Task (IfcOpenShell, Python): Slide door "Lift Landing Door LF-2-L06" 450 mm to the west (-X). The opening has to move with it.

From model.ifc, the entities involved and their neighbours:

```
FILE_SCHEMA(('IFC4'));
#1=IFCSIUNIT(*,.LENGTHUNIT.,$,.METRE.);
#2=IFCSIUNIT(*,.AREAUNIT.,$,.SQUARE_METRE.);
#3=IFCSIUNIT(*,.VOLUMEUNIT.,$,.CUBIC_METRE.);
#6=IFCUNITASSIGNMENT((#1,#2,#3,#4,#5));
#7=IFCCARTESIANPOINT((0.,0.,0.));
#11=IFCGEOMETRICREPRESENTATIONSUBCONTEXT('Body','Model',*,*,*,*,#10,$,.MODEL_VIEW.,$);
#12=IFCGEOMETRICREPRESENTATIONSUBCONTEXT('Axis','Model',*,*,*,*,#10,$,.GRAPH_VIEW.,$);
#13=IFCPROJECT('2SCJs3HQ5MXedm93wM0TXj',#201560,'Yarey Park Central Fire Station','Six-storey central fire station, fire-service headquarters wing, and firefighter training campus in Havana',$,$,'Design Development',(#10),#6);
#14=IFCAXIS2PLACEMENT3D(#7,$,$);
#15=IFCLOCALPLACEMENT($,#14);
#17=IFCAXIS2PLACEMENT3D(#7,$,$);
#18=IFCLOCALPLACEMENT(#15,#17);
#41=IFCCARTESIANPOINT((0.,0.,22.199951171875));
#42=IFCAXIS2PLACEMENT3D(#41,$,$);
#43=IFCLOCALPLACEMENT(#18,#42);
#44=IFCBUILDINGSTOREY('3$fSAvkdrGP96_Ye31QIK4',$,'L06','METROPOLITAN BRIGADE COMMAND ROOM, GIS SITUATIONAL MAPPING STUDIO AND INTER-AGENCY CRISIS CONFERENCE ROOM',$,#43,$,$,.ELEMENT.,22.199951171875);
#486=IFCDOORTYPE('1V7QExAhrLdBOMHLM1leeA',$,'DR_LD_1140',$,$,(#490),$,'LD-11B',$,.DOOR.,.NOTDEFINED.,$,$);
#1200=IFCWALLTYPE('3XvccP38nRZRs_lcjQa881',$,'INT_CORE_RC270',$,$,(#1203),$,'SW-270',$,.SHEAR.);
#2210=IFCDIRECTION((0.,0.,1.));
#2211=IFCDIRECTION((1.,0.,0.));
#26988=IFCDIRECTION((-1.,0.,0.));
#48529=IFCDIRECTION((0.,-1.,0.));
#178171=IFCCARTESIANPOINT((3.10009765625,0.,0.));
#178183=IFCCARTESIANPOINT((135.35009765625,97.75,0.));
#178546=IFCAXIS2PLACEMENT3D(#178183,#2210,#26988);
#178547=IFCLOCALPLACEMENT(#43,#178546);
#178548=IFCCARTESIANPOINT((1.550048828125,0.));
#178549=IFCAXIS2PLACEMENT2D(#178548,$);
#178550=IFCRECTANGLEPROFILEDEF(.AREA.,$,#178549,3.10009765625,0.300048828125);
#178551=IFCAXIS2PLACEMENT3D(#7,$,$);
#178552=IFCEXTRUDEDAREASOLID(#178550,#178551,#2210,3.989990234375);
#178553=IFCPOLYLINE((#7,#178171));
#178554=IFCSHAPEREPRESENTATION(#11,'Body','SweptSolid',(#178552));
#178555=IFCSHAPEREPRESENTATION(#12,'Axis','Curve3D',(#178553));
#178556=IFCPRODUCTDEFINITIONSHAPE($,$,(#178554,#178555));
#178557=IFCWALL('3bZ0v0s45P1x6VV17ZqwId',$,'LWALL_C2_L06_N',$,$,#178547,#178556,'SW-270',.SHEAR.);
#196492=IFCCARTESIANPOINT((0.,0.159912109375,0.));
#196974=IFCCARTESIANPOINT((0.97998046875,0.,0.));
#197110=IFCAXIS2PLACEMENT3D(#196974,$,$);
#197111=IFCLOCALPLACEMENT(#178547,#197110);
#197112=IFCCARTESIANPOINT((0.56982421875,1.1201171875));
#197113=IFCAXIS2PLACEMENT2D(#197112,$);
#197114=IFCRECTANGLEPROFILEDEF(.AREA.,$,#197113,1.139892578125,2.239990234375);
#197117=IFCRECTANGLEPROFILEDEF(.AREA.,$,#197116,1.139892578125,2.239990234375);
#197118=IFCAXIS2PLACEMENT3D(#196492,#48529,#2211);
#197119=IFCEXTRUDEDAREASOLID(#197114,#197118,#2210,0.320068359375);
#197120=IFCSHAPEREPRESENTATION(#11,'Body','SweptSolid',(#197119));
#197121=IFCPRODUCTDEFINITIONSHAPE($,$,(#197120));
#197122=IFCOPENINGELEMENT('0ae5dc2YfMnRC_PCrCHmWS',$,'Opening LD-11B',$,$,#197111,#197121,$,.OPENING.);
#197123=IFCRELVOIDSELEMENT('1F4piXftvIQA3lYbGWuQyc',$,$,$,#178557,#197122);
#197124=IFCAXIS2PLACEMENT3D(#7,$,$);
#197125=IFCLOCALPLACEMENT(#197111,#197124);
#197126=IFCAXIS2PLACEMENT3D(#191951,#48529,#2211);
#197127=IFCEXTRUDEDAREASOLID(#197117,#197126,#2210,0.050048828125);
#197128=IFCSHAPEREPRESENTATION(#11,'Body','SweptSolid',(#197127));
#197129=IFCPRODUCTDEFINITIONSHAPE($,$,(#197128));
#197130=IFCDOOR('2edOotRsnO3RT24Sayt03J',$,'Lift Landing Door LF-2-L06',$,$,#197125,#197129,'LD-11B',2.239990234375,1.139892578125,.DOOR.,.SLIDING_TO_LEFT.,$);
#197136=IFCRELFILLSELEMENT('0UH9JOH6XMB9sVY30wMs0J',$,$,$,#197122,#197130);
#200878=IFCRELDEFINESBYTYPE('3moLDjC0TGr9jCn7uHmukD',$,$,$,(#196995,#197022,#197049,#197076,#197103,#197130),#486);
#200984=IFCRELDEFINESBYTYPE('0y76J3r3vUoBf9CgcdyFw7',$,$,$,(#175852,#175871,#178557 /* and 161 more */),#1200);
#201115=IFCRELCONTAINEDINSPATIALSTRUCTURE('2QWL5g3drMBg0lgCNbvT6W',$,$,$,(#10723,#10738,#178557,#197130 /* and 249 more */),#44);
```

```python
import ifcopenshell
import ifcopenshell.api.geometry
import ifcopenshell.util.placement
import ifcopenshell.util.unit

model = ifcopenshell.open("model.ifc")
unit_scale = ifcopenshell.util.unit.calculate_unit_scale(model)

door = model.by_guid("2edOotRsnO3RT24Sayt03J")
opening = door.FillsVoids[0].RelatingOpeningElement
wall = opening.VoidsElements[0].RelatingBuildingElement

wall_matrix = ifcopenshell.util.placement.get_local_placement(wall.ObjectPlacement)
shift = wall_matrix[:3, 0] * 0.45 / unit_scale
before = ifcopenshell.util.placement.get_local_placement(door.ObjectPlacement)[:3, 3].copy()

# The door is placed relative to its opening, so it follows when the opening moves.
matrix = ifcopenshell.util.placement.get_local_placement(opening.ObjectPlacement)
matrix[:3, 3] += shift
ifcopenshell.api.geometry.edit_object_placement(
    model, product=opening, matrix=matrix, is_si=False, should_transform_children=True
)

after = ifcopenshell.util.placement.get_local_placement(door.ObjectPlacement)[:3, 3]
print("door moved by", (after - before).round(3) + 0.0)

model.write("model_v2.ifc")
```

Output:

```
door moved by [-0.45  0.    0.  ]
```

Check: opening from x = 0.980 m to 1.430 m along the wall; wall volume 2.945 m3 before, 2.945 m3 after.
